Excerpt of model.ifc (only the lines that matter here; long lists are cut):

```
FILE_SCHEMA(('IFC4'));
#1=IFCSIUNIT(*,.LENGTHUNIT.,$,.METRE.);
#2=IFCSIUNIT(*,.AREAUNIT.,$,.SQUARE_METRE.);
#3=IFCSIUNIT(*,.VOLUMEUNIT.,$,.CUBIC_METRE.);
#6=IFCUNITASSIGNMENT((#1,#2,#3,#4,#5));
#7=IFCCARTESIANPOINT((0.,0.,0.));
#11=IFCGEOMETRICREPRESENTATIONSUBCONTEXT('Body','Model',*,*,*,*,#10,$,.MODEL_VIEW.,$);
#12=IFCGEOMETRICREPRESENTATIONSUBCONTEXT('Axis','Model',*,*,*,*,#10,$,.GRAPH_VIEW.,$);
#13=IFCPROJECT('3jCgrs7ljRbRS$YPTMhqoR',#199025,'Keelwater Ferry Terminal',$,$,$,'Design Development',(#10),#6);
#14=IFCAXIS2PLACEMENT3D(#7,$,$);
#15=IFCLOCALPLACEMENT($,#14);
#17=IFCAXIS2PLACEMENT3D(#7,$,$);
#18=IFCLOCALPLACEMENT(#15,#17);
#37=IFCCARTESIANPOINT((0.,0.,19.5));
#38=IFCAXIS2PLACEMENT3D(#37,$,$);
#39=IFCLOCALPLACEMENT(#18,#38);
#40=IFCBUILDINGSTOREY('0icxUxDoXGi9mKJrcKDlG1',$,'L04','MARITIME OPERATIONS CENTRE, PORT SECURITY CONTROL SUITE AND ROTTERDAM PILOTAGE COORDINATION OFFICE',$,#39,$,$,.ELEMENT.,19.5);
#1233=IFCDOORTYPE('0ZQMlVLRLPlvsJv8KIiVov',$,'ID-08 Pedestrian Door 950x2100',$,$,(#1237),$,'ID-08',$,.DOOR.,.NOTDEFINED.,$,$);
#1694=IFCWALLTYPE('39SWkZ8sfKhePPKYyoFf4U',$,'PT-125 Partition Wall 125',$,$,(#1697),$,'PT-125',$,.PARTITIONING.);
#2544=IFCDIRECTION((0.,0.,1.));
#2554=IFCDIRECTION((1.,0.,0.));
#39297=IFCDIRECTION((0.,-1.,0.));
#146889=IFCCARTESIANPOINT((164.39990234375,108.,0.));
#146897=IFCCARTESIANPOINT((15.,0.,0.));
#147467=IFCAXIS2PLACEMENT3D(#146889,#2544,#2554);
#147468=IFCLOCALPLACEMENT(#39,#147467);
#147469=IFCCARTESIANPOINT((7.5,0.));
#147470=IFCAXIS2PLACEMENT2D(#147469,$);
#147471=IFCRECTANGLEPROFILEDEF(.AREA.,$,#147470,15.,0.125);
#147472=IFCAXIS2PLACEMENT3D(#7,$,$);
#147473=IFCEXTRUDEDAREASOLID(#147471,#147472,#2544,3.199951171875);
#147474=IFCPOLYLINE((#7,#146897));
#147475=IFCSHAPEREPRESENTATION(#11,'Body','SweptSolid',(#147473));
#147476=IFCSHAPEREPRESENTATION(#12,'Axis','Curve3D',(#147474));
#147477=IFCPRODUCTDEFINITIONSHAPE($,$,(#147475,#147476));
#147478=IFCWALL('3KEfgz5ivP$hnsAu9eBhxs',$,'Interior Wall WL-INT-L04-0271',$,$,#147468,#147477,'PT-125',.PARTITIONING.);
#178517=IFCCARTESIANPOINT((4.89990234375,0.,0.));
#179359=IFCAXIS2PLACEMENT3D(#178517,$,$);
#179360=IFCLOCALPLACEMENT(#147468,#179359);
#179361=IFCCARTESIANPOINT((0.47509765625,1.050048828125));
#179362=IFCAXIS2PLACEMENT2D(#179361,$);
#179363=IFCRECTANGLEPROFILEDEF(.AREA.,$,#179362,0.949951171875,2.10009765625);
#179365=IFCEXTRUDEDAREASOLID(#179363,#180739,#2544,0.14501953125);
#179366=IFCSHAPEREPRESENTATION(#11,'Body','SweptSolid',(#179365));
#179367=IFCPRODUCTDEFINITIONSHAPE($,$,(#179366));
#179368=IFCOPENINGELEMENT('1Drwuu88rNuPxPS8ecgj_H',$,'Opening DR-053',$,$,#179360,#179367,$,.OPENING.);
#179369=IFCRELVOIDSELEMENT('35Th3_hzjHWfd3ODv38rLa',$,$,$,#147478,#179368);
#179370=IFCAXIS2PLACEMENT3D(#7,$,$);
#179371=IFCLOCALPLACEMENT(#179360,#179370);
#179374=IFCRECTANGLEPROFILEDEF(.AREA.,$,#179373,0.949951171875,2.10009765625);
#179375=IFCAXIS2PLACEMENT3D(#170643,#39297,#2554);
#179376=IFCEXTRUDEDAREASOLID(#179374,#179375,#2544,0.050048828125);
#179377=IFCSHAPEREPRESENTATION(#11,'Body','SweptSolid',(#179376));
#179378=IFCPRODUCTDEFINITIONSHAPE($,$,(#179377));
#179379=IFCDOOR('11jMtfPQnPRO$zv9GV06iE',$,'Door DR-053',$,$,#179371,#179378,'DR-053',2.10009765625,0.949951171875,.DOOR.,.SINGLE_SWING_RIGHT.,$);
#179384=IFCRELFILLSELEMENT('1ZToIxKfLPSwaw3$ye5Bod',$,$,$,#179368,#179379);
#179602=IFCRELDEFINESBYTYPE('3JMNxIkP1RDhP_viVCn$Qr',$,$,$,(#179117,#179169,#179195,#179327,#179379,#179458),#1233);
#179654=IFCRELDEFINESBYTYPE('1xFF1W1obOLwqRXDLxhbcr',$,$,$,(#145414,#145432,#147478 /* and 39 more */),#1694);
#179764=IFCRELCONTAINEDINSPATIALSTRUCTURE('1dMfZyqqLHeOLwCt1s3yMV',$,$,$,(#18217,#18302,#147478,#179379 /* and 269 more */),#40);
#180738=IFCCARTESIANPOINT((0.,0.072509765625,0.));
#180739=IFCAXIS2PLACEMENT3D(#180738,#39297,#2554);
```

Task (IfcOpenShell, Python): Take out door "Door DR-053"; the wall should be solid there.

```python
import ifcopenshell
import ifcopenshell.api.feature
import ifcopenshell.api.root
import ifcopenshell.geom
import ifcopenshell.util.shape

model = ifcopenshell.open("model.ifc")
settings = ifcopenshell.geom.settings()


def volume(element):
    """Net volume in cubic metres, openings subtracted."""
    shape = ifcopenshell.geom.create_shape(settings, element)
    return ifcopenshell.util.shape.get_volume(shape.geometry)


door = model.by_guid("11jMtfPQnPRO$zv9GV06iE")
opening = door.FillsVoids[0].RelatingOpeningElement
wall = opening.VoidsElements[0].RelatingBuildingElement
before = volume(wall)

ifcopenshell.api.root.remove_product(model, product=door)
ifcopenshell.api.feature.remove_feature(model, feature=opening)

after = volume(wall)

print(f"wall volume {before:.3f} -> {after:.3f} m3")

model.write("model_updated.ifc")
```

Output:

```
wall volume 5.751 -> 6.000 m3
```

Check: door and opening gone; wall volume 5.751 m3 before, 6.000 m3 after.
